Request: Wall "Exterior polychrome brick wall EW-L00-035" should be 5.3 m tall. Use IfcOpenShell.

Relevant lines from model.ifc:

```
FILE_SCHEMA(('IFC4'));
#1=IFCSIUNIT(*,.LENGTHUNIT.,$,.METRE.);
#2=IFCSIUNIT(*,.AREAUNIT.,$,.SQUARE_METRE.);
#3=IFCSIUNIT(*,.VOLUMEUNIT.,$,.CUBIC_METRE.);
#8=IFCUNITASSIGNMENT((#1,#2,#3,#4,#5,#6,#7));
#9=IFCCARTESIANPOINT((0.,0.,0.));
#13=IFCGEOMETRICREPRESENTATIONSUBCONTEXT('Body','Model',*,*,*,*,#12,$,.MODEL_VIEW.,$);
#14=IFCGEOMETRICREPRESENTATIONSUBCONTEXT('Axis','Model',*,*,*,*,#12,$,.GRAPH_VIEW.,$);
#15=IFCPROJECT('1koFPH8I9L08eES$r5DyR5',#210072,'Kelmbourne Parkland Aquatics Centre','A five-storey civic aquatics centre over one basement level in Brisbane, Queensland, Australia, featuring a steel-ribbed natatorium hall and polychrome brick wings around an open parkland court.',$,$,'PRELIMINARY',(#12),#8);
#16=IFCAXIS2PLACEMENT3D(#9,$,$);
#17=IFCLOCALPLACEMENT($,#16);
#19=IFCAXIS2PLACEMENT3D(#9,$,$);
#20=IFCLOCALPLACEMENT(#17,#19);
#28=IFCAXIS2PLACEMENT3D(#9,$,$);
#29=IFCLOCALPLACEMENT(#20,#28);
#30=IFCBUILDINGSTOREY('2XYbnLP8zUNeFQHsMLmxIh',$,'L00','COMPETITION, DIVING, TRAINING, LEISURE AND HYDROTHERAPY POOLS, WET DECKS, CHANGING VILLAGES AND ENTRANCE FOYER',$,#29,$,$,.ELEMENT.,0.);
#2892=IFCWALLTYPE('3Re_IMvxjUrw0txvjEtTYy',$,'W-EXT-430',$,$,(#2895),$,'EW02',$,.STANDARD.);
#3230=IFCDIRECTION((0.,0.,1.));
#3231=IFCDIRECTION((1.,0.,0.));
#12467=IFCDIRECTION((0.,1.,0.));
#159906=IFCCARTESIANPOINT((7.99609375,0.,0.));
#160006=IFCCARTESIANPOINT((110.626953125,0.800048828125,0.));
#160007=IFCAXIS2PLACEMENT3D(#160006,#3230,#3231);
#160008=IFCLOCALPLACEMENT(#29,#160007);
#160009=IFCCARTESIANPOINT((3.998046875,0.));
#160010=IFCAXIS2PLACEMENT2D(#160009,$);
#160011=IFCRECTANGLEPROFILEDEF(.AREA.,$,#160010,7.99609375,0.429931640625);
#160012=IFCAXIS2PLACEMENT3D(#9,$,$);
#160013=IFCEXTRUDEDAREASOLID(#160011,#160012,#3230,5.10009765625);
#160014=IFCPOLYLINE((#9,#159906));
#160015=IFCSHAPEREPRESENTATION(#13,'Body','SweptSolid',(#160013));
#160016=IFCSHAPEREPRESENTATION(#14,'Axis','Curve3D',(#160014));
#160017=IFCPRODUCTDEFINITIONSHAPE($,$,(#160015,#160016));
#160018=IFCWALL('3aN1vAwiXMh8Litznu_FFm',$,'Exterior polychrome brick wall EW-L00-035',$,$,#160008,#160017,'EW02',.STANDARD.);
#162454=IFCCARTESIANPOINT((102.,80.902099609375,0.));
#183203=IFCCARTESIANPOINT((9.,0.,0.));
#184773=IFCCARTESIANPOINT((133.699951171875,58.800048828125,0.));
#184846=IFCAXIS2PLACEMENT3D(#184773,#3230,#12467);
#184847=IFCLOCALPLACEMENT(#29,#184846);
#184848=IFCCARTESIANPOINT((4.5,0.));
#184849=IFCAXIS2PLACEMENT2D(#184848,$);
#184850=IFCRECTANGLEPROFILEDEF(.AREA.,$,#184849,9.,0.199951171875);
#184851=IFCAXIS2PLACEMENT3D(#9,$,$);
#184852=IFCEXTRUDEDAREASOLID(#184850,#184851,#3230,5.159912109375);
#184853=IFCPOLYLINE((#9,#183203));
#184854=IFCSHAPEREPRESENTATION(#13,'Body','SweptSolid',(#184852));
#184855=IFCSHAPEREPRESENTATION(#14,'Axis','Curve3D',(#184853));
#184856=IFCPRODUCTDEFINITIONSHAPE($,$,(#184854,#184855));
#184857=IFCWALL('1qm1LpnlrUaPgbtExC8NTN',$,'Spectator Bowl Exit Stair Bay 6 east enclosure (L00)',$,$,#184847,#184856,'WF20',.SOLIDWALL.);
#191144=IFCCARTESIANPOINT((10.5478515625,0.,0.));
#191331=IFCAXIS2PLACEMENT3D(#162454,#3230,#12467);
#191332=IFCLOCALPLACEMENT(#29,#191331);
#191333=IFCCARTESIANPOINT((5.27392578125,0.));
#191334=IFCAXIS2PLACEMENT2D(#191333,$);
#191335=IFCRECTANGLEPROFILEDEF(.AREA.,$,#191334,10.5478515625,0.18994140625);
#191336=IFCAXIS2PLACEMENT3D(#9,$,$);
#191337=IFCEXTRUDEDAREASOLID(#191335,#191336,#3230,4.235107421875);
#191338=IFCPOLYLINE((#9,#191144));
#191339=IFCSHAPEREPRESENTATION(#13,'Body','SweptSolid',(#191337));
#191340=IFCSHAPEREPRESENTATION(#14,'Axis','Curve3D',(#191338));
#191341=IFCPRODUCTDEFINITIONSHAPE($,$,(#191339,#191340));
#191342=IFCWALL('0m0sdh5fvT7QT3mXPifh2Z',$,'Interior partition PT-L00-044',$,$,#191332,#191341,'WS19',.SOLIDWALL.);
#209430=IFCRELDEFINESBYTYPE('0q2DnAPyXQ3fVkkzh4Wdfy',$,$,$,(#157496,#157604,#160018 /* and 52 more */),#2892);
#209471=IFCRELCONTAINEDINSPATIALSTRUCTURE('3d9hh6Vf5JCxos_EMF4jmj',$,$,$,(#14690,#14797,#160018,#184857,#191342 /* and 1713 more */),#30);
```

```python
import ifcopenshell
import ifcopenshell.geom
import ifcopenshell.util.representation
import ifcopenshell.util.shape
import ifcopenshell.util.unit

model = ifcopenshell.open("model.ifc")
unit_scale = ifcopenshell.util.unit.calculate_unit_scale(model)
settings = ifcopenshell.geom.settings()


def volume(element):
    """Net volume in cubic metres, openings subtracted."""
    shape = ifcopenshell.geom.create_shape(settings, element)
    return ifcopenshell.util.shape.get_volume(shape.geometry)


wall = model.by_guid("3aN1vAwiXMh8Litznu_FFm")
before = volume(wall)

body = ifcopenshell.util.representation.get_representation(wall, "Model", "Body")
solid = body.Items[0]
old_height = solid.Depth
solid.Depth = 5.3 / unit_scale
after = volume(wall)

print(f"height {old_height:g} -> {solid.Depth:g}, volume {before:.3f} -> {after:.3f} m3")

model.write("model-out.ifc")
```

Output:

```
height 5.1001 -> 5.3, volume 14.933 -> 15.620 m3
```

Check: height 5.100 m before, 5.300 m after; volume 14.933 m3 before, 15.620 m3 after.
